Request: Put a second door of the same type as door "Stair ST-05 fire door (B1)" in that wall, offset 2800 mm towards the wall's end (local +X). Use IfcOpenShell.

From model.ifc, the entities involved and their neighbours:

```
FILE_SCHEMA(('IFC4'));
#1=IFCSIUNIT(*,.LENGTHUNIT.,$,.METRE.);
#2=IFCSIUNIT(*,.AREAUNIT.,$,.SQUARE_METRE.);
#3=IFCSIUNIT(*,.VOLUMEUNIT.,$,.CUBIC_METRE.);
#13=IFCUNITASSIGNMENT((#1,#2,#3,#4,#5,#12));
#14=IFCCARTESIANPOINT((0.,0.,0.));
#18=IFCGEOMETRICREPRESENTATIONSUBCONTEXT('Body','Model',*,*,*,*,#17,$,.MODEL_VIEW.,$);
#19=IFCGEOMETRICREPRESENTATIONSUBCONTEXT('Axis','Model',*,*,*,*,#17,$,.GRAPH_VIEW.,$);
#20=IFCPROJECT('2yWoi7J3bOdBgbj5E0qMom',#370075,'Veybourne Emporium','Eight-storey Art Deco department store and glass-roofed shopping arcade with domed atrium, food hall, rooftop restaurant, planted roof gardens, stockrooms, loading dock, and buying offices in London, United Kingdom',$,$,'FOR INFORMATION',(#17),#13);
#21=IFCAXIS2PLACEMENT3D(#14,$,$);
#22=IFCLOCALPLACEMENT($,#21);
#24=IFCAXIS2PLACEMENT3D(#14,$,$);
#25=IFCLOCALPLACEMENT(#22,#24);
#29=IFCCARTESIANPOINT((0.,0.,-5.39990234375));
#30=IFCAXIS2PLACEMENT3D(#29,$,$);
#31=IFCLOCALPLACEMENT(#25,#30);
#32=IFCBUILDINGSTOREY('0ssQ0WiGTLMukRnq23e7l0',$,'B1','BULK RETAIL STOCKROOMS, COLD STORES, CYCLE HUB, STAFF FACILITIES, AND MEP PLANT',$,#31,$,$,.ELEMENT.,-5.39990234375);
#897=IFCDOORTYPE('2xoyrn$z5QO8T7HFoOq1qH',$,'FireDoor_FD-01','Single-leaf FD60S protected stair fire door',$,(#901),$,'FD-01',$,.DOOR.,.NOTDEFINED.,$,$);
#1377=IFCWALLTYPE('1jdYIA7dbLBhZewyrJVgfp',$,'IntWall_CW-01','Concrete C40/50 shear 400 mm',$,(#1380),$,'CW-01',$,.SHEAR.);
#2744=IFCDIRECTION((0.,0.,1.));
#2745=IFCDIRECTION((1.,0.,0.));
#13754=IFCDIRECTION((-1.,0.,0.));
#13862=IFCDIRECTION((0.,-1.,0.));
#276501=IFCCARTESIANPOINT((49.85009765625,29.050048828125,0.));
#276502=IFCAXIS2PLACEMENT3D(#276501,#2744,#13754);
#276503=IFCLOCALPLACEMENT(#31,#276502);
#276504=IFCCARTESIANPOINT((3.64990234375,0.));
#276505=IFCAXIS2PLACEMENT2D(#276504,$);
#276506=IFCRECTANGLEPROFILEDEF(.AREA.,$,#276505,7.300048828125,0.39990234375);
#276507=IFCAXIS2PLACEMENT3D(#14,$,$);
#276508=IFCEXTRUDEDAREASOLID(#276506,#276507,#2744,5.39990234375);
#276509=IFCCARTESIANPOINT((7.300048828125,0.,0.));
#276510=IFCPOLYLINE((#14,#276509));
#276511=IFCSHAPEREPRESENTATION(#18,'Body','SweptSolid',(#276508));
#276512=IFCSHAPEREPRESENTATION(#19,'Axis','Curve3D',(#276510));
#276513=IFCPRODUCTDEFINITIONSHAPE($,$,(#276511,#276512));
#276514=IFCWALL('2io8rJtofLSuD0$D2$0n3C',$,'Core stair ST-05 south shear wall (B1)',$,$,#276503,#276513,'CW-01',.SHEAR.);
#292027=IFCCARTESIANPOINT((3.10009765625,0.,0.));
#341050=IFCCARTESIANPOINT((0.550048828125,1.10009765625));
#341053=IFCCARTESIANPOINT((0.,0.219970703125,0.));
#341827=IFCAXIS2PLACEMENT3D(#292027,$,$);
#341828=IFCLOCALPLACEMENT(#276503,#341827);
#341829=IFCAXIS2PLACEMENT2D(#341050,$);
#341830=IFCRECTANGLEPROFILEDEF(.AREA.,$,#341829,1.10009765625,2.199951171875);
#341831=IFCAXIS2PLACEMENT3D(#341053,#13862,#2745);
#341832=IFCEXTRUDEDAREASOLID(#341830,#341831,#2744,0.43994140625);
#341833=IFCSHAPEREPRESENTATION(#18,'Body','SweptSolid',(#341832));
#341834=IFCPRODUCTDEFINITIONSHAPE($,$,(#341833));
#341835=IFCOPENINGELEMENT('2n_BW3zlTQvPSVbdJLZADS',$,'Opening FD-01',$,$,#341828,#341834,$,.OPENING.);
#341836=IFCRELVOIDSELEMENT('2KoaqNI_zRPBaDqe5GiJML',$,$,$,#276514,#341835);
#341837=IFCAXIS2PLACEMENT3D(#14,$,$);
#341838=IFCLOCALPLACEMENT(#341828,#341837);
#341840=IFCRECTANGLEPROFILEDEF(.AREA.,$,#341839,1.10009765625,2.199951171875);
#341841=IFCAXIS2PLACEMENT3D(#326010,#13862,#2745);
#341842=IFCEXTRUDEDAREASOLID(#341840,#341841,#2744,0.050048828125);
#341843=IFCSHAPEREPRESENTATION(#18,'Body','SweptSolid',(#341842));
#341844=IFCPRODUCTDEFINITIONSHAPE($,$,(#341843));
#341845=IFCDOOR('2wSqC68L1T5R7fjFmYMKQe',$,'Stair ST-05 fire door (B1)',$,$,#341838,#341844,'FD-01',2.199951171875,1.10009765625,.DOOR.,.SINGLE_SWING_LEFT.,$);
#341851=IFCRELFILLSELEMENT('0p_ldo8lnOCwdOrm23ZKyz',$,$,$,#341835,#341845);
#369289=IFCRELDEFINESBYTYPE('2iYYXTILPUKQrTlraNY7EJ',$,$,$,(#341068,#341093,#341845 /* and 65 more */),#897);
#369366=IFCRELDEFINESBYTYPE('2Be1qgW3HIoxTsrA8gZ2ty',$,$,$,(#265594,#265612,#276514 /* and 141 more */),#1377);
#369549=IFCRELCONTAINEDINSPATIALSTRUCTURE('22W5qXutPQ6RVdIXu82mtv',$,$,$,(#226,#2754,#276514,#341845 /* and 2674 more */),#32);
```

```python
import ifcopenshell
import ifcopenshell.api.feature
import ifcopenshell.api.geometry
import ifcopenshell.api.root
import ifcopenshell.geom
import ifcopenshell.util.element
import ifcopenshell.util.placement
import ifcopenshell.util.shape

model = ifcopenshell.open("model.ifc")
settings = ifcopenshell.geom.settings()


def volume(element):
    """Net volume in cubic metres, openings subtracted."""
    shape = ifcopenshell.geom.create_shape(settings, element)
    return ifcopenshell.util.shape.get_volume(shape.geometry)


door = model.by_guid("2wSqC68L1T5R7fjFmYMKQe")
opening = door.FillsVoids[0].RelatingOpeningElement
wall = opening.VoidsElements[0].RelatingBuildingElement
before = volume(wall)
shift = ifcopenshell.util.placement.get_local_placement(wall.ObjectPlacement)[:3, 0] * 2.8

# copy_class copies the void relationship, type, container and properties, but no geometry.
new_opening = ifcopenshell.api.root.copy_class(model, product=opening)
new_opening.Representation = ifcopenshell.util.element.copy_deep(
    model, opening.Representation, exclude=["IfcGeometricRepresentationContext", "IfcRepresentationMap"]
)
new_door = ifcopenshell.api.root.copy_class(model, product=door)
new_door.Representation = ifcopenshell.util.element.copy_deep(
    model, door.Representation, exclude=["IfcGeometricRepresentationContext", "IfcRepresentationMap"]
)
new_door.Tag = None
ifcopenshell.api.feature.add_filling(model, opening=new_opening, element=new_door)

for old, new in ((opening, new_opening), (door, new_door)):
    matrix = ifcopenshell.util.placement.get_local_placement(old.ObjectPlacement)
    matrix[:3, 3] += shift
    ifcopenshell.api.geometry.edit_object_placement(model, product=new, matrix=matrix, is_si=False)

after = volume(wall)

print(f"wall volume {before:.3f} -> {after:.3f} m3")

model.write("model_edited.ifc")
```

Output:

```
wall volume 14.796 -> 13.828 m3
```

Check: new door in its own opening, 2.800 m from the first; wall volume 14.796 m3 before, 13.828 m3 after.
